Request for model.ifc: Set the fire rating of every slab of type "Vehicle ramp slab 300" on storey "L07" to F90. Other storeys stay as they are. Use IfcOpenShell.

First a look at what the model holds.

```python
import ifcopenshell
import ifcopenshell.util.element

model = ifcopenshell.open("model.ifc")
print(model.schema)
storey = next(s for s in model.by_type("IfcBuildingStorey") if s.Name == "L07")
slabs = [e for e in ifcopenshell.util.element.get_decomposition(storey) if e.is_a("IfcSlab")]
seen = {}
for e in slabs:
    element_type = ifcopenshell.util.element.get_type(e)
    key = (element_type.Name if element_type != e and element_type else None, ifcopenshell.util.element.get_pset(e, "Pset_SlabCommon", "FireRating"))
    seen[key] = seen.get(key, 0) + 1
for (name, value), count in sorted(seen.items(), key=str):
    print(count, "x", name, "|", value)
```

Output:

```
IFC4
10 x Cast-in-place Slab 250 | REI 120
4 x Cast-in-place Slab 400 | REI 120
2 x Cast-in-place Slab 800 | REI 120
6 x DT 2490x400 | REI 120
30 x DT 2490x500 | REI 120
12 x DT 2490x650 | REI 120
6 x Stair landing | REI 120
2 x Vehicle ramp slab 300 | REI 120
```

```python
import ifcopenshell
import ifcopenshell.api.pset
import ifcopenshell.util.element

model = ifcopenshell.open("model.ifc")

storey = next(s for s in model.by_type("IfcBuildingStorey") if s.Name == "L07")
slabs = [e for e in ifcopenshell.util.element.get_decomposition(storey) if e.is_a("IfcSlab")]

count = 0
for e in slabs:
    element_type = ifcopenshell.util.element.get_type(e)
    if element_type in (None, e) or element_type.Name != "Vehicle ramp slab 300":
        continue
    # add_pset returns the element's existing set when there is one.
    pset = ifcopenshell.api.pset.add_pset(model, product=e, name="Pset_SlabCommon")
    ifcopenshell.api.pset.edit_pset(model, pset=pset, properties={"FireRating": "F90"})
    count += 1

print(count, "slabs updated")

model.write("model_updated.ifc")
```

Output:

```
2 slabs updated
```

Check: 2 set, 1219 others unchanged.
